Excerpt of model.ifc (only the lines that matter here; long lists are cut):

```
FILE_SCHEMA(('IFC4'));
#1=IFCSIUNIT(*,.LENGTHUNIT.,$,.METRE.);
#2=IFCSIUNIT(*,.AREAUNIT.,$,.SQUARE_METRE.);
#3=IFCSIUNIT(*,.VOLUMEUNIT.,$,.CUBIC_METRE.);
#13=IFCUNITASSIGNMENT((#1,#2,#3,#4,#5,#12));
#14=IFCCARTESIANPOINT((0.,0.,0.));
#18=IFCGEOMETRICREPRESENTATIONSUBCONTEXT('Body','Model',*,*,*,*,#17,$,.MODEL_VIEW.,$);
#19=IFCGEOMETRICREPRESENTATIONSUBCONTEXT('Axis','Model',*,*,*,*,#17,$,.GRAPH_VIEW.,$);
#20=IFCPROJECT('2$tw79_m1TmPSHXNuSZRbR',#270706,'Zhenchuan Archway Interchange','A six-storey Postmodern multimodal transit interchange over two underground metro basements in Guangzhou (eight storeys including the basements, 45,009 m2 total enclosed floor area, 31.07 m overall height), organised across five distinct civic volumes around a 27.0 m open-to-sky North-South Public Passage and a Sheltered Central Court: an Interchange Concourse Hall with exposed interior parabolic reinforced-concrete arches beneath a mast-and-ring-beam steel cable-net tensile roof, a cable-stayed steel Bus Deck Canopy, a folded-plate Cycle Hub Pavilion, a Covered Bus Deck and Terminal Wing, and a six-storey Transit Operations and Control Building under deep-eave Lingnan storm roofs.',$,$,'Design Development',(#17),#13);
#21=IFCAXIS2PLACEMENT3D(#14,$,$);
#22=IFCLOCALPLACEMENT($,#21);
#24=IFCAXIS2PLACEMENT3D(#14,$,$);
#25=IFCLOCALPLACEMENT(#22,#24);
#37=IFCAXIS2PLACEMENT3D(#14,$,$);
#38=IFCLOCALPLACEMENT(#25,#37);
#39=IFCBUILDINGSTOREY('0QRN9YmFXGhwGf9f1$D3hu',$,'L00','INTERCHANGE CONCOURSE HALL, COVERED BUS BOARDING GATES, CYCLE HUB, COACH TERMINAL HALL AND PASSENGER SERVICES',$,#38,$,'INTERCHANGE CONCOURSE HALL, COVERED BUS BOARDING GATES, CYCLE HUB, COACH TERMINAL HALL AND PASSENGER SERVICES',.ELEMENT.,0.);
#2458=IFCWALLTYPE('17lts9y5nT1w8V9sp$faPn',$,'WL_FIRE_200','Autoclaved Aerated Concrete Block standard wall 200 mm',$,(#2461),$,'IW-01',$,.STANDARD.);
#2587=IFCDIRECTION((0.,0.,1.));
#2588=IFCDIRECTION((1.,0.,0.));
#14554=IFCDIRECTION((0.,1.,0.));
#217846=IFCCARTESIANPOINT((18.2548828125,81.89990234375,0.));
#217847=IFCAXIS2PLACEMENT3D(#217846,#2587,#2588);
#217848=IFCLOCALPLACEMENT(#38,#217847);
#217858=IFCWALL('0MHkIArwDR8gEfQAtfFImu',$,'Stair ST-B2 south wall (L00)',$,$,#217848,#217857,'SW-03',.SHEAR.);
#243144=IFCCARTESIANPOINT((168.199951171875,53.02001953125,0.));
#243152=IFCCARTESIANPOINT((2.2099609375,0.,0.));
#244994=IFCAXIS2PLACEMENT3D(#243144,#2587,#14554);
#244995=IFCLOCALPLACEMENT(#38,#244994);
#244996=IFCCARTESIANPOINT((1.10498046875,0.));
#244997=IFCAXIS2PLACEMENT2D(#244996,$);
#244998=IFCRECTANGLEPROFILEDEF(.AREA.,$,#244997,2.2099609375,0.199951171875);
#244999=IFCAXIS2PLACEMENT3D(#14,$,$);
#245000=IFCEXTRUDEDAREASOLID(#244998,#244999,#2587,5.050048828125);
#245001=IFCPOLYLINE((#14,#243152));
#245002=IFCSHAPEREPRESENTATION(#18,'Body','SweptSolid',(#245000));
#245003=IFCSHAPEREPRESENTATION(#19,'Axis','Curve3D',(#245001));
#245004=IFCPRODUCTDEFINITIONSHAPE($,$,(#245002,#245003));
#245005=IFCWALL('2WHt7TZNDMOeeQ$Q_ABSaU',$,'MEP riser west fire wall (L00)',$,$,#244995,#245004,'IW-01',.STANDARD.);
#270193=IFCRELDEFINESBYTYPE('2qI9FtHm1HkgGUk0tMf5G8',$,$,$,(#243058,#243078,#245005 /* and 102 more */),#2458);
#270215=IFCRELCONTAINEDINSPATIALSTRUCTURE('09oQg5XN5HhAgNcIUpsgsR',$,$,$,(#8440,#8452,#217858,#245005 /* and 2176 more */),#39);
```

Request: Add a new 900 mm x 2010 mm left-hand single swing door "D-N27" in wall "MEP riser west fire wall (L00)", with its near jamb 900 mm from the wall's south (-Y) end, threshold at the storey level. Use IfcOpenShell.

```python
import numpy as np
import ifcopenshell
import ifcopenshell.api.feature
import ifcopenshell.api.geometry
import ifcopenshell.api.root
import ifcopenshell.api.spatial
import ifcopenshell.geom
import ifcopenshell.util.element
import ifcopenshell.util.placement
import ifcopenshell.util.representation
import ifcopenshell.util.shape
import ifcopenshell.util.unit

model = ifcopenshell.open("model.ifc")
unit_scale = ifcopenshell.util.unit.calculate_unit_scale(model)
settings = ifcopenshell.geom.settings()


def volume(element):
    """Net volume in cubic metres, openings subtracted."""
    shape = ifcopenshell.geom.create_shape(settings, element)
    return ifcopenshell.util.shape.get_volume(shape.geometry)


wall = model.by_guid("2WHt7TZNDMOeeQ$Q_ABSaU")
storey = ifcopenshell.util.element.get_container(wall, ifc_class="IfcBuildingStorey")
context = ifcopenshell.util.representation.get_context(model, "Model", "Body", "MODEL_VIEW")
before = volume(wall)

width, height, from_end, sill = 0.9, 2.01, 0.9, 0.0  # metres

# The wall runs along its own X axis, and the end named is its -X end.
wall_shape = ifcopenshell.geom.create_shape(settings, wall)
x, y, z = ifcopenshell.util.shape.get_vertices(wall_shape.geometry).T
start = x.min() + from_end
face, thickness = float(y.min()), float(y.max() - y.min())
wall_matrix = ifcopenshell.util.placement.get_local_placement(wall.ObjectPlacement)
level = ifcopenshell.util.placement.get_local_placement(storey.ObjectPlacement)[2, 3]


def in_wall(x, y):
    """Placement at x, y metres in the wall's axes, at sill height."""
    matrix = wall_matrix.copy()
    matrix[:, 3] = wall_matrix @ np.array([x / unit_scale, y / unit_scale, 0.0, 1.0])
    matrix[2, 3] = level + sill / unit_scale
    return matrix


# Opening: a box that overshoots both wall faces by 50 mm.
opening = ifcopenshell.api.root.create_entity(model, ifc_class="IfcOpeningElement", predefined_type="OPENING")
box = ifcopenshell.api.geometry.add_wall_representation(
    model, context=context, length=width, height=height, thickness=thickness + 0.1
)
ifcopenshell.api.geometry.assign_representation(model, product=opening, representation=box)
ifcopenshell.api.geometry.edit_object_placement(model, product=opening, matrix=in_wall(start, face - 0.05), is_si=False)
ifcopenshell.api.feature.add_feature(model, feature=opening, element=wall)

door = ifcopenshell.api.root.create_entity(model, ifc_class="IfcDoor", name="D-N27", predefined_type="DOOR")
door.OverallWidth, door.OverallHeight = width / unit_scale, height / unit_scale
door.OperationType = "SINGLE_SWING_LEFT"
body = ifcopenshell.api.geometry.add_door_representation(
    model,
    context=context,
    overall_width=door.OverallWidth,
    overall_height=door.OverallHeight,
    operation_type="SINGLE_SWING_LEFT",
    lining_properties={"LiningDepth": thickness / unit_scale, "ThresholdDepth": thickness / unit_scale},
)
ifcopenshell.api.geometry.assign_representation(model, product=door, representation=body)
ifcopenshell.api.spatial.assign_container(model, products=[door], relating_structure=storey)
ifcopenshell.api.feature.add_filling(model, opening=opening, element=door)

# The lining spans the wall, so the door starts at the wall face.
ifcopenshell.api.geometry.edit_object_placement(model, product=door, matrix=in_wall(start, face), is_si=False)

after = volume(wall)

print(f"wall volume {before:.3f} -> {after:.3f} m3")

model.write("model_v2.ifc")
```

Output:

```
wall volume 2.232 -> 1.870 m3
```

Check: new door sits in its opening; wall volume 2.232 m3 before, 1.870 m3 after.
